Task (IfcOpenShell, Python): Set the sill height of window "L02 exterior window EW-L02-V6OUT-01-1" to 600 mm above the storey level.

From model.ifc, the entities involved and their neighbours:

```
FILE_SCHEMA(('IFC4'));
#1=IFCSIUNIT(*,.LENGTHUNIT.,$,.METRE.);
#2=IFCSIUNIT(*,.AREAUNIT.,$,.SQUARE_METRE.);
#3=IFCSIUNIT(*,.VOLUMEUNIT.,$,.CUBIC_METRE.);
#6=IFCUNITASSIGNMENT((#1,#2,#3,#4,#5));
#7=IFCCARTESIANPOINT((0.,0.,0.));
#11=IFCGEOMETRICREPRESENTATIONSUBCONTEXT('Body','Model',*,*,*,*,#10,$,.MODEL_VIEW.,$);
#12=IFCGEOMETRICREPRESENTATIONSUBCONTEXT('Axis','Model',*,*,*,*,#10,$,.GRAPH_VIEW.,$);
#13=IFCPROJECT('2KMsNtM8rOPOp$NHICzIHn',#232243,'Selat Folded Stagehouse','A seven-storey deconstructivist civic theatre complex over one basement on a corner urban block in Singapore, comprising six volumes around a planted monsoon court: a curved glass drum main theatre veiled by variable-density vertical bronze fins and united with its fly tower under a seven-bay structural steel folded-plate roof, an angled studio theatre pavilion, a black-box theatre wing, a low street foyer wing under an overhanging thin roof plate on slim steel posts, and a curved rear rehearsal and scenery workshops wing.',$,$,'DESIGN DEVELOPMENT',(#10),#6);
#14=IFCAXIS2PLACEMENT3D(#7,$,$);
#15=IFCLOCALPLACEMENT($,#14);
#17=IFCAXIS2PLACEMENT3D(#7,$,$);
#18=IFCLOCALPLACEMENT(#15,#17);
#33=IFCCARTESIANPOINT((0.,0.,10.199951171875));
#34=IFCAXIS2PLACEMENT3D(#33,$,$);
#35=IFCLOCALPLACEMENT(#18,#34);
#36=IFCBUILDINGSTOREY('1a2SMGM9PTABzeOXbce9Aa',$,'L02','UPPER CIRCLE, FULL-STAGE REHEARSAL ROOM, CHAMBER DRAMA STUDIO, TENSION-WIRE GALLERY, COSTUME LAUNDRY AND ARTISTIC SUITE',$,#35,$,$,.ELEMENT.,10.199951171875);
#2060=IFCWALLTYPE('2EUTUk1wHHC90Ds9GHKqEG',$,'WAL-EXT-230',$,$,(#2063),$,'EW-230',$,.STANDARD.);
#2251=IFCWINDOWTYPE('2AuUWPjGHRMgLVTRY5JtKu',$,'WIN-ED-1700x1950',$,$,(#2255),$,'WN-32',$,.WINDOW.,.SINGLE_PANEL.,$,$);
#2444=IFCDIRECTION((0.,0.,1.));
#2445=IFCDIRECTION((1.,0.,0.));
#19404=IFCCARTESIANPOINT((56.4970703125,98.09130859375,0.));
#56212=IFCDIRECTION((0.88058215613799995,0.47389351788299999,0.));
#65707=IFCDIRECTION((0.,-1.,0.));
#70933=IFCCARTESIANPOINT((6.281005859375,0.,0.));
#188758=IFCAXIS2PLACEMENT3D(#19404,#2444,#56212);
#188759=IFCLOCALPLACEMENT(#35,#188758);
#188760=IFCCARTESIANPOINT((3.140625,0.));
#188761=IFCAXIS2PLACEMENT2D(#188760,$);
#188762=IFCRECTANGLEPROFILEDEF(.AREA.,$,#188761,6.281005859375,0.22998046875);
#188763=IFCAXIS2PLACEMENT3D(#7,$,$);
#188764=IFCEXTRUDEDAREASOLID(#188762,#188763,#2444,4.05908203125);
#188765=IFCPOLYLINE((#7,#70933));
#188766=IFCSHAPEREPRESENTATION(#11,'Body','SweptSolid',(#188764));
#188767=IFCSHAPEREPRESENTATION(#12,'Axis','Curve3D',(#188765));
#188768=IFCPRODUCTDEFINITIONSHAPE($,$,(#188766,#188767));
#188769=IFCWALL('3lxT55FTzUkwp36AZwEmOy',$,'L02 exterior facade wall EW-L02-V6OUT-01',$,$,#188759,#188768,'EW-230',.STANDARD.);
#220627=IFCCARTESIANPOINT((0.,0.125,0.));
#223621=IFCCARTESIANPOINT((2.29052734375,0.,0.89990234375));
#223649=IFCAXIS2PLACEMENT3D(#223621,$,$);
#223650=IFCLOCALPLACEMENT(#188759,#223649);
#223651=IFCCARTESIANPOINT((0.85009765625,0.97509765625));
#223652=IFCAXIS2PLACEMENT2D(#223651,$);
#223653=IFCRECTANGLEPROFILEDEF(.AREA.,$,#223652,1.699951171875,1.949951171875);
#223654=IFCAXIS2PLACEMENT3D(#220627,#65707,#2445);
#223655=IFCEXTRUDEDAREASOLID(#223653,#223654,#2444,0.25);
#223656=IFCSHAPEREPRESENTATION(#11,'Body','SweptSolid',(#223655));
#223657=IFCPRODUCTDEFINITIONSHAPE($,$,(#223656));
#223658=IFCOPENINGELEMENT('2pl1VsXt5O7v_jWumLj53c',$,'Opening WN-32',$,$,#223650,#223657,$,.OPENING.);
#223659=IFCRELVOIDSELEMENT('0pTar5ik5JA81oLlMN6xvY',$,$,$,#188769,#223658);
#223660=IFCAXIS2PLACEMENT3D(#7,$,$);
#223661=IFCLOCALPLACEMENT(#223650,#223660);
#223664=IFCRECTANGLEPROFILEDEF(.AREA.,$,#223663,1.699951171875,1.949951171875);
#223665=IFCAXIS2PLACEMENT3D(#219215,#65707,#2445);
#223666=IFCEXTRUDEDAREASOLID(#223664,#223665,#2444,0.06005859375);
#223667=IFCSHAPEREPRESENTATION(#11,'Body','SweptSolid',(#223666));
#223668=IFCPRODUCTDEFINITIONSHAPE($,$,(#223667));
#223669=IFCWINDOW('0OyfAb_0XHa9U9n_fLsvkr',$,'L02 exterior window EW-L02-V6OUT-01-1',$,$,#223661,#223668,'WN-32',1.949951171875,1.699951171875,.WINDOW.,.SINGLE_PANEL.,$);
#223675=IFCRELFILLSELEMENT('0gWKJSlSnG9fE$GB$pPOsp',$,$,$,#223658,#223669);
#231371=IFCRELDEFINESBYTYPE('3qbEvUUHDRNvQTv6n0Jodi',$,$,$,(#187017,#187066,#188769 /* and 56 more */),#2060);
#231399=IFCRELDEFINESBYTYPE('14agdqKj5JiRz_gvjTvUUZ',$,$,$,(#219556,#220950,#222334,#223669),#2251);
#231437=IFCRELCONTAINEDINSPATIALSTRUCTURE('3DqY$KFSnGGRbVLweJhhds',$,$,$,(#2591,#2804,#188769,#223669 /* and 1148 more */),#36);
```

```python
import numpy as np
import ifcopenshell
import ifcopenshell.api.geometry
import ifcopenshell.geom
import ifcopenshell.util.element
import ifcopenshell.util.placement
import ifcopenshell.util.shape
import ifcopenshell.util.unit

model = ifcopenshell.open("model.ifc")
unit_scale = ifcopenshell.util.unit.calculate_unit_scale(model)

window = model.by_guid("0OyfAb_0XHa9U9n_fLsvkr")
opening = window.FillsVoids[0].RelatingOpeningElement
storey = ifcopenshell.util.element.get_container(window, ifc_class="IfcBuildingStorey")
level = ifcopenshell.util.placement.get_local_placement(storey.ObjectPlacement)[2, 3]

# The opening's origin need not be at the sill, so measure its lowest point.
shape = ifcopenshell.geom.create_shape(ifcopenshell.geom.settings(), opening)
bottom = ifcopenshell.util.shape.get_shape_bottom_elevation(shape, shape.geometry) / unit_scale
dz = level + 0.6 / unit_scale - bottom

shift = np.array([0.0, 0.0, dz])
# The window is placed relative to its opening, so it follows when the opening moves.
matrix = ifcopenshell.util.placement.get_local_placement(opening.ObjectPlacement)
matrix[:3, 3] += shift
ifcopenshell.api.geometry.edit_object_placement(
    model, product=opening, matrix=matrix, is_si=False, should_transform_children=True
)

print(f"moved by {dz * unit_scale:+.3f} m")

model.write("model_edited.ifc")
```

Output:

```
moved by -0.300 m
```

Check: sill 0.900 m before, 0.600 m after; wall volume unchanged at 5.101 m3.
